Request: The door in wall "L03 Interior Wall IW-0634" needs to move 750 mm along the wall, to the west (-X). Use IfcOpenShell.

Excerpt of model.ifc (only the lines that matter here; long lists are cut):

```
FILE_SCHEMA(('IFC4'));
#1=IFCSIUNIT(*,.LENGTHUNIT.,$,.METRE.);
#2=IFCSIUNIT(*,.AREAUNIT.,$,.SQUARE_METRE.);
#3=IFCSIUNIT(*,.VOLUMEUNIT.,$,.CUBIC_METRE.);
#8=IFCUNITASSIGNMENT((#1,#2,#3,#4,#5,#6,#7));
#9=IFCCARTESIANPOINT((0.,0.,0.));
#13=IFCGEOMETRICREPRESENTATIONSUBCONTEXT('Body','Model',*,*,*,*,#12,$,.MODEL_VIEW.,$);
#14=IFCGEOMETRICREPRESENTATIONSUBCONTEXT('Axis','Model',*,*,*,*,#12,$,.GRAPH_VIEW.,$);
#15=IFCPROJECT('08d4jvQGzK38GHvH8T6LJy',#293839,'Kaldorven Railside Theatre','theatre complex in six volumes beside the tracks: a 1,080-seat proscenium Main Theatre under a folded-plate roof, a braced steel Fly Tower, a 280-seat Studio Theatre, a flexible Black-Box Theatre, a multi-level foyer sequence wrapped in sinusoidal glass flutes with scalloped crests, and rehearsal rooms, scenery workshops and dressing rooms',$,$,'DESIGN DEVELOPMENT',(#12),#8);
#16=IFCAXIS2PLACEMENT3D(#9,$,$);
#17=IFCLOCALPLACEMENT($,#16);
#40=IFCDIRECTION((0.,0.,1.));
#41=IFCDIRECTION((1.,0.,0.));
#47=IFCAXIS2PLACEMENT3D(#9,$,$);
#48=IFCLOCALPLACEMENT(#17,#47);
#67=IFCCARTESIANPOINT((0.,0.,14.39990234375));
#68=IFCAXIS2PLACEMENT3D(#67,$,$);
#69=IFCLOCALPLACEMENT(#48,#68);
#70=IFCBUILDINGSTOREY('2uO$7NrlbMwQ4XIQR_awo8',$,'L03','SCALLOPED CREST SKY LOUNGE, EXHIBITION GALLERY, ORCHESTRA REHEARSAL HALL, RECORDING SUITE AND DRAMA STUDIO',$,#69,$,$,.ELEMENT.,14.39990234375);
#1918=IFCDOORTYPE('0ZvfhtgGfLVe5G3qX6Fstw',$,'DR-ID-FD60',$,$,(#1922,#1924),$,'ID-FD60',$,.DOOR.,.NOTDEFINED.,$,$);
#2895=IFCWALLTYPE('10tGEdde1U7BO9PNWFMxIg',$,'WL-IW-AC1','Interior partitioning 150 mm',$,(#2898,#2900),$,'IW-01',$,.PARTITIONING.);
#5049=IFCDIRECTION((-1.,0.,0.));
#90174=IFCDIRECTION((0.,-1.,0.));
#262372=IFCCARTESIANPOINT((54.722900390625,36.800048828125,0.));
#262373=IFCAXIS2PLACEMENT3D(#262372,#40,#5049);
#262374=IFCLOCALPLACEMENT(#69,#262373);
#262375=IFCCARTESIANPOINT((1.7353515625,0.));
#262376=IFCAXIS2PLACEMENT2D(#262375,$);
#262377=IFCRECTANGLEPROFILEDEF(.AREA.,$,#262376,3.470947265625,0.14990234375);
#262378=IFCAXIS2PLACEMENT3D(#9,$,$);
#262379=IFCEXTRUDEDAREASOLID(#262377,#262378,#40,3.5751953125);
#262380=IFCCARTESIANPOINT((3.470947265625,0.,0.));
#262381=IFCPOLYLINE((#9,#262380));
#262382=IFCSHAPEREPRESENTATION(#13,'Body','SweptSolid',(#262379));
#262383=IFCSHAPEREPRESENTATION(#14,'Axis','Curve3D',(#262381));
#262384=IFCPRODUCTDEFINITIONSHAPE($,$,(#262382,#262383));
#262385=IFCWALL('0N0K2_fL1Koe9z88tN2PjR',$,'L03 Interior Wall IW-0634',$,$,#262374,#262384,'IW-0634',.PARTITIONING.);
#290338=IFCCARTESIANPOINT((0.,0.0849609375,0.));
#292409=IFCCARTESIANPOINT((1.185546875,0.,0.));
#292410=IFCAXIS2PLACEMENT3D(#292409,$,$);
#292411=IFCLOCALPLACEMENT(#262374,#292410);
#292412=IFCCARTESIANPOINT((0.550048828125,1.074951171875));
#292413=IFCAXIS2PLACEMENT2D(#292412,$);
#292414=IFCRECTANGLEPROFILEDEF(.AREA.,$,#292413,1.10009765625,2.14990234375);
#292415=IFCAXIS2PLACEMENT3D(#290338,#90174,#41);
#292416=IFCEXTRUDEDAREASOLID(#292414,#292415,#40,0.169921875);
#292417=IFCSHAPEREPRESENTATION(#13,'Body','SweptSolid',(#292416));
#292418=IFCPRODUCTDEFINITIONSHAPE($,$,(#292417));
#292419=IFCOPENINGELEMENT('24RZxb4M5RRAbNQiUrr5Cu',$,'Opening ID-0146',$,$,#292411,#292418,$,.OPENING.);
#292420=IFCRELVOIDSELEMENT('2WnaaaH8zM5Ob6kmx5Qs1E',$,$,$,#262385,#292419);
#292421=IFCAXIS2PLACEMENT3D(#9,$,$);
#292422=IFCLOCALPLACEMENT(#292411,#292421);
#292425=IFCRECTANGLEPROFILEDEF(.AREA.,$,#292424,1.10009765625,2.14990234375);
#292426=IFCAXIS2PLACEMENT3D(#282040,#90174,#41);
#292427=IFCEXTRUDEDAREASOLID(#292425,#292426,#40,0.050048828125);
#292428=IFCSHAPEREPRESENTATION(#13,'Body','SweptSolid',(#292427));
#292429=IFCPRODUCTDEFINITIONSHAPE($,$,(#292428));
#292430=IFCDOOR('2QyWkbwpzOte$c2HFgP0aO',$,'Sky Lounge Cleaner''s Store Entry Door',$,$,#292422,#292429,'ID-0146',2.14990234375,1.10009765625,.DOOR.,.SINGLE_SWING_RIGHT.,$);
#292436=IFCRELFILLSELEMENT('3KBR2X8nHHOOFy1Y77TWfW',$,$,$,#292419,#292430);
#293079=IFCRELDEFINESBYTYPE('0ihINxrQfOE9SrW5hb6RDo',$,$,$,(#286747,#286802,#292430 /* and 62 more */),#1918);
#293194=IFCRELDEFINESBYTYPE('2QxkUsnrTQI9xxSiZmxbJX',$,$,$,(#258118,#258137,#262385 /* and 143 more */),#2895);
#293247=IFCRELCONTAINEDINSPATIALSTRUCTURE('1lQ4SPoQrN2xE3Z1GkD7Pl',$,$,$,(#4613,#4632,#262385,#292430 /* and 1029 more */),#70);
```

```python
import ifcopenshell
import ifcopenshell.api.geometry
import ifcopenshell.util.placement
import ifcopenshell.util.unit

model = ifcopenshell.open("model.ifc")
unit_scale = ifcopenshell.util.unit.calculate_unit_scale(model)

door = model.by_guid("2QyWkbwpzOte$c2HFgP0aO")
opening = door.FillsVoids[0].RelatingOpeningElement
wall = opening.VoidsElements[0].RelatingBuildingElement

wall_matrix = ifcopenshell.util.placement.get_local_placement(wall.ObjectPlacement)
shift = wall_matrix[:3, 0] * 0.75 / unit_scale
before = ifcopenshell.util.placement.get_local_placement(door.ObjectPlacement)[:3, 3].copy()

# The door is placed relative to its opening, so it follows when the opening moves.
matrix = ifcopenshell.util.placement.get_local_placement(opening.ObjectPlacement)
matrix[:3, 3] += shift
ifcopenshell.api.geometry.edit_object_placement(
    model, product=opening, matrix=matrix, is_si=False, should_transform_children=True
)

after = ifcopenshell.util.placement.get_local_placement(door.ObjectPlacement)[:3, 3]
print("door moved by", (after - before).round(3) + 0.0)

model.write("model_rev.ifc")
```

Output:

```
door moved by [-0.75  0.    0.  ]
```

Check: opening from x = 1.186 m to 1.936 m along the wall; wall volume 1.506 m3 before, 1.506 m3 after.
